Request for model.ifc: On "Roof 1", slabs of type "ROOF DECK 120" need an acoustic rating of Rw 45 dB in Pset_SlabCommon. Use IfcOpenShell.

First a look at what the model holds.

```python
import ifcopenshell
import ifcopenshell.util.element

model = ifcopenshell.open("model.ifc")
print(model.schema)
storey = next(s for s in model.by_type("IfcBuildingStorey") if s.Name == "Roof 1")
slabs = [e for e in ifcopenshell.util.element.get_decomposition(storey) if e.is_a("IfcSlab")]
seen = {}
for e in slabs:
    element_type = ifcopenshell.util.element.get_type(e)
    key = (element_type.Name if element_type != e and element_type else None, ifcopenshell.util.element.get_pset(e, "Pset_SlabCommon", "AcousticRating"))
    seen[key] = seen.get(key, 0) + 1
for (name, value), count in sorted(seen.items(), key=str):
    print(count, "x", name, "|", value)
```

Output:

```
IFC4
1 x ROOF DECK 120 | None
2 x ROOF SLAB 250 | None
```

```python
import ifcopenshell
import ifcopenshell.api.pset
import ifcopenshell.util.element

model = ifcopenshell.open("model.ifc")

storey = next(s for s in model.by_type("IfcBuildingStorey") if s.Name == "Roof 1")
slabs = [e for e in ifcopenshell.util.element.get_decomposition(storey) if e.is_a("IfcSlab")]

count = 0
for e in slabs:
    element_type = ifcopenshell.util.element.get_type(e)
    if element_type in (None, e) or element_type.Name != "ROOF DECK 120":
        continue
    # add_pset returns the element's existing set when there is one.
    pset = ifcopenshell.api.pset.add_pset(model, product=e, name="Pset_SlabCommon")
    ifcopenshell.api.pset.edit_pset(model, pset=pset, properties={"AcousticRating": "Rw 45 dB"})
    count += 1

print(count, "slabs updated")

model.write("model_updated.ifc")
```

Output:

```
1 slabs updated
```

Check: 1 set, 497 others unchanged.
